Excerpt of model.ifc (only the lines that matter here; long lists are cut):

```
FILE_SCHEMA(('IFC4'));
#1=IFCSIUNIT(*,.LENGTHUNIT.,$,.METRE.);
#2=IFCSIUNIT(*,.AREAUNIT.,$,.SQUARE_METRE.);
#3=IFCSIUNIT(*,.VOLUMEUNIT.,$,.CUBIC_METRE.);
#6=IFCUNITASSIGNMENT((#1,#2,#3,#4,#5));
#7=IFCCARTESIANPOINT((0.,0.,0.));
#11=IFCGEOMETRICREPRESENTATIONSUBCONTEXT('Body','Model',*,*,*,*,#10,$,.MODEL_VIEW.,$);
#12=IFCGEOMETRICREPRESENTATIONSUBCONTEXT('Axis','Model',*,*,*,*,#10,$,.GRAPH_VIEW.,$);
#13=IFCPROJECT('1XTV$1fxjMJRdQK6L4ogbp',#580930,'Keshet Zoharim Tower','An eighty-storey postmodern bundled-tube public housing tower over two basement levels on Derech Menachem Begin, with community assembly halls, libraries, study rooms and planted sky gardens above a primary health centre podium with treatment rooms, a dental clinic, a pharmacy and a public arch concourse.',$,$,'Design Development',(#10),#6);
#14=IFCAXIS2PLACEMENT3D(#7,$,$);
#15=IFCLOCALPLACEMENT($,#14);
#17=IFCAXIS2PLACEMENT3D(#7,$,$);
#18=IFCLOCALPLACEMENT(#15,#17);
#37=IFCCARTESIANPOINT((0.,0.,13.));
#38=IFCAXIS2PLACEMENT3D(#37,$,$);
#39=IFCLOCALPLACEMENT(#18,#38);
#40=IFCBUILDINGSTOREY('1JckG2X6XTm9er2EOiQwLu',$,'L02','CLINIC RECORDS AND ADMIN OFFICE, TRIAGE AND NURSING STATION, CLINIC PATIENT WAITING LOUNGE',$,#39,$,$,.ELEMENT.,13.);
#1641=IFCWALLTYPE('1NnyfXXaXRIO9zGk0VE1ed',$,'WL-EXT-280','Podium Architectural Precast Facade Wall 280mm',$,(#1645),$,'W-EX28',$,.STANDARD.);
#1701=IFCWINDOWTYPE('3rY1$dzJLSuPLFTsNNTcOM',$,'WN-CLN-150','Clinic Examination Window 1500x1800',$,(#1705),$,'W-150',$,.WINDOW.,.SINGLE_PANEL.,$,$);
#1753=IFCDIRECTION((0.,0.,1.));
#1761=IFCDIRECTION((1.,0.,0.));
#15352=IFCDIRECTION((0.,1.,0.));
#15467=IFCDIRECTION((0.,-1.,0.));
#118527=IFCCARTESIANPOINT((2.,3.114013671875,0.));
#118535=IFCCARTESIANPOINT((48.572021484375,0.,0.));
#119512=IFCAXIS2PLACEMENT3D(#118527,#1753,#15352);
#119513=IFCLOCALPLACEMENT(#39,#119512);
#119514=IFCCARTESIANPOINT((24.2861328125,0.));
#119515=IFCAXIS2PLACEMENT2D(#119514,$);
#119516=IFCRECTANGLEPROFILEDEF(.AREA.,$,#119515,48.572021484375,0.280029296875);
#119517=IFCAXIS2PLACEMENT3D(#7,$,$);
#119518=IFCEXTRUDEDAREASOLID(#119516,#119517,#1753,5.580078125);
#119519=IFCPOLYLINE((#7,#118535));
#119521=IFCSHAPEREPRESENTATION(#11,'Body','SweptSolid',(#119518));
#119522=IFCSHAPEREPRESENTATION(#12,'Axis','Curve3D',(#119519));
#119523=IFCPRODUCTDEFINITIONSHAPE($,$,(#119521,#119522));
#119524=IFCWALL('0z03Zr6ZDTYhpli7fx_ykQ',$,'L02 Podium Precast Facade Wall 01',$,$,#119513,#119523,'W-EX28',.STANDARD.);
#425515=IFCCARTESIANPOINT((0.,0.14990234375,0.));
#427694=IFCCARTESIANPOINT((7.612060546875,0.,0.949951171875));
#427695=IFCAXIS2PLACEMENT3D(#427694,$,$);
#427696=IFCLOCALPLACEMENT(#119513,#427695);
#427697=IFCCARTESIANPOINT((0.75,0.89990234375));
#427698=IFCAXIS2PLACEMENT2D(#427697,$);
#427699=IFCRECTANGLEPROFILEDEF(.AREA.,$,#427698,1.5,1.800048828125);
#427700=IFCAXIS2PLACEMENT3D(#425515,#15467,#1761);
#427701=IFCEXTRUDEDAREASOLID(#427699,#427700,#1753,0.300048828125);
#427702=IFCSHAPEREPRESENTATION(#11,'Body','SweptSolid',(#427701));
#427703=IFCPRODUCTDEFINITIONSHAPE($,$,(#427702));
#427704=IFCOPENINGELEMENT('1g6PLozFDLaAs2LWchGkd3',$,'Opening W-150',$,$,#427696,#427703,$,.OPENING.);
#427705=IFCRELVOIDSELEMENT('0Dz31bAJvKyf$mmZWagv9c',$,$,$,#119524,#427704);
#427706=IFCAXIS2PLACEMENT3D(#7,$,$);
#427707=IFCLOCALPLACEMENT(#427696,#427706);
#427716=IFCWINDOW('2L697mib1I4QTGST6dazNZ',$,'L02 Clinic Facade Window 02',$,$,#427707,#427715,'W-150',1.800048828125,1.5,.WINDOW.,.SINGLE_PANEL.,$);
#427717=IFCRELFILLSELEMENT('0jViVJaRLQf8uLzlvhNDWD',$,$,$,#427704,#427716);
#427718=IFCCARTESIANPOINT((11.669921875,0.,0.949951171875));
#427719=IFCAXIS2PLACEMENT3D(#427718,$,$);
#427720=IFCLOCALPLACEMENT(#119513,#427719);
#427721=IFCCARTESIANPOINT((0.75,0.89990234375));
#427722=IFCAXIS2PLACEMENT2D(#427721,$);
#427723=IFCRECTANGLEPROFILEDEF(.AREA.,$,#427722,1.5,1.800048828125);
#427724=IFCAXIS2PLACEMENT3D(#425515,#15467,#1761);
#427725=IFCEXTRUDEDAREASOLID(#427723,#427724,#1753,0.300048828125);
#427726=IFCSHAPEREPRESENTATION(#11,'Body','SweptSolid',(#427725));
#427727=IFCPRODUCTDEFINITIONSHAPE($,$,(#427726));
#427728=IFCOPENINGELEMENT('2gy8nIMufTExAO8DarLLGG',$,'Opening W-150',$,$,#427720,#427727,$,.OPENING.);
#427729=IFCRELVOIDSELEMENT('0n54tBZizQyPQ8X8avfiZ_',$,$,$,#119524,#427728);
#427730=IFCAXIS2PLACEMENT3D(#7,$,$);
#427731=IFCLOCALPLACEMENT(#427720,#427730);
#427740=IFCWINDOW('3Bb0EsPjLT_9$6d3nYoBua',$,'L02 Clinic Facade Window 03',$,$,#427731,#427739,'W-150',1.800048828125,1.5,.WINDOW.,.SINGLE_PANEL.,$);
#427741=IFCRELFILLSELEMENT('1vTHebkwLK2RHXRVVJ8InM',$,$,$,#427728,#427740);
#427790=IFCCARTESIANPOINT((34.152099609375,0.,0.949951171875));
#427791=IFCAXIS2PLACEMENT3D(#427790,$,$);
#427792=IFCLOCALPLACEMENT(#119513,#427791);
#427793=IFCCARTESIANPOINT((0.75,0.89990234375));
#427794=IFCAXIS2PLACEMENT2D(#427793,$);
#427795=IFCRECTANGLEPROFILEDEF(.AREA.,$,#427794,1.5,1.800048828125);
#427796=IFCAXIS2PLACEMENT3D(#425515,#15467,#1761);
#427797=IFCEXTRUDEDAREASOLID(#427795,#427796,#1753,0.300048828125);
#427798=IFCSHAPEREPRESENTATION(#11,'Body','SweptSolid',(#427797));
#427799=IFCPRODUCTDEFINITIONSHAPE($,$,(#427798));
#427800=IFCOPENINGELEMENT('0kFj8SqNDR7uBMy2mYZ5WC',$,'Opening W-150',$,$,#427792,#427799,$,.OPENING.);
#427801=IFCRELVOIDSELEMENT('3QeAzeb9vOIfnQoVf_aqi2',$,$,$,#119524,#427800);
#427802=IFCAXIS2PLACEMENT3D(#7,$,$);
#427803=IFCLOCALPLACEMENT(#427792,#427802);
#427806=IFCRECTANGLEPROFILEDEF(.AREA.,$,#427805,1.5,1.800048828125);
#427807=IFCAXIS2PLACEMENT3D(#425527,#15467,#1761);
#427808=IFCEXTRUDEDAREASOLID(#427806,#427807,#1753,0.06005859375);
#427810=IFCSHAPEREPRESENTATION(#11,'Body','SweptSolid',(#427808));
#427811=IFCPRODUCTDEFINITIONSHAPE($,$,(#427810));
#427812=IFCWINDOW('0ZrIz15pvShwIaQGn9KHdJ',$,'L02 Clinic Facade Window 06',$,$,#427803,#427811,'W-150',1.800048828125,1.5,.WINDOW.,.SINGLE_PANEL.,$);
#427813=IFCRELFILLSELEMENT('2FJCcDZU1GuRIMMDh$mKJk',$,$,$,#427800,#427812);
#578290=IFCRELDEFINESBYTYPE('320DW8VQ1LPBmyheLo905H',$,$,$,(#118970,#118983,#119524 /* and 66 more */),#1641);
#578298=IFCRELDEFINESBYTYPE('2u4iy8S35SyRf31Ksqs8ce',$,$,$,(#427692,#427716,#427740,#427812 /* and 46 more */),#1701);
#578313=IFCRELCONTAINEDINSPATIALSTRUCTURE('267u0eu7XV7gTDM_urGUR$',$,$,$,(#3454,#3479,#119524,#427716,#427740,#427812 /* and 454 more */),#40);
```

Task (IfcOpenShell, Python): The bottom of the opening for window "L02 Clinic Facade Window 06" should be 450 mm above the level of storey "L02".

```python
import numpy as np
import ifcopenshell
import ifcopenshell.api.geometry
import ifcopenshell.geom
import ifcopenshell.util.element
import ifcopenshell.util.placement
import ifcopenshell.util.shape
import ifcopenshell.util.unit

model = ifcopenshell.open("model.ifc")
unit_scale = ifcopenshell.util.unit.calculate_unit_scale(model)

window = model.by_guid("0ZrIz15pvShwIaQGn9KHdJ")
opening = window.FillsVoids[0].RelatingOpeningElement
storey = ifcopenshell.util.element.get_container(window, ifc_class="IfcBuildingStorey")
level = ifcopenshell.util.placement.get_local_placement(storey.ObjectPlacement)[2, 3]

# The opening's origin need not be at the sill, so measure its lowest point.
shape = ifcopenshell.geom.create_shape(ifcopenshell.geom.settings(), opening)
bottom = ifcopenshell.util.shape.get_shape_bottom_elevation(shape, shape.geometry) / unit_scale
dz = level + 0.45 - bottom

shift = np.array([0.0, 0.0, dz])
# The window is placed relative to its opening, so it follows when the opening moves.
matrix = ifcopenshell.util.placement.get_local_placement(opening.ObjectPlacement)
matrix[:3, 3] += shift
ifcopenshell.api.geometry.edit_object_placement(
    model, product=opening, matrix=matrix, is_si=False, should_transform_children=True
)

print(f"moved by {dz * unit_scale:+.3f} m")

model.write("model_updated.ifc")
```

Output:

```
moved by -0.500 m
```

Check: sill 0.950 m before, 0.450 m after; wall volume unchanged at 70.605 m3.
